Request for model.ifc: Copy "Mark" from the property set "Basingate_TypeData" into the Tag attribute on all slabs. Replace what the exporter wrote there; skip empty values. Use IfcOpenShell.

First a look at what the model holds.

```python
import ifcopenshell
import ifcopenshell.util.element

model = ifcopenshell.open("model.ifc")
print(model.schema)
slabs = model.by_type("IfcSlab")
print(len(slabs), "slabs")
for e in slabs[:8]:
    source = ifcopenshell.util.element.get_pset(e, "Basingate_TypeData", "Mark")
    target = e.Tag
    print(e.id(), repr(source), repr(target), sep=" | ")
```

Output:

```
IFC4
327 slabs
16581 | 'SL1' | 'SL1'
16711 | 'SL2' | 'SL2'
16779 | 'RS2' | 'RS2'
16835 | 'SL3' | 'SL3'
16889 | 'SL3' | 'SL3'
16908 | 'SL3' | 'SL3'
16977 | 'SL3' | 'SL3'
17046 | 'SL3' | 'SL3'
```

```python
import ifcopenshell
import ifcopenshell.util.element

model = ifcopenshell.open("model.ifc")

count = 0
for e in model.by_type("IfcSlab"):
    value = ifcopenshell.util.element.get_pset(e, "Basingate_TypeData", "Mark")
    current = e.Tag
    if not value or not value.strip() or current == value:
        continue
    e.Tag = value
    count += 1

print(count, "slabs updated")

model.write("model_updated.ifc")
```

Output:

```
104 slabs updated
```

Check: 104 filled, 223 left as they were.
